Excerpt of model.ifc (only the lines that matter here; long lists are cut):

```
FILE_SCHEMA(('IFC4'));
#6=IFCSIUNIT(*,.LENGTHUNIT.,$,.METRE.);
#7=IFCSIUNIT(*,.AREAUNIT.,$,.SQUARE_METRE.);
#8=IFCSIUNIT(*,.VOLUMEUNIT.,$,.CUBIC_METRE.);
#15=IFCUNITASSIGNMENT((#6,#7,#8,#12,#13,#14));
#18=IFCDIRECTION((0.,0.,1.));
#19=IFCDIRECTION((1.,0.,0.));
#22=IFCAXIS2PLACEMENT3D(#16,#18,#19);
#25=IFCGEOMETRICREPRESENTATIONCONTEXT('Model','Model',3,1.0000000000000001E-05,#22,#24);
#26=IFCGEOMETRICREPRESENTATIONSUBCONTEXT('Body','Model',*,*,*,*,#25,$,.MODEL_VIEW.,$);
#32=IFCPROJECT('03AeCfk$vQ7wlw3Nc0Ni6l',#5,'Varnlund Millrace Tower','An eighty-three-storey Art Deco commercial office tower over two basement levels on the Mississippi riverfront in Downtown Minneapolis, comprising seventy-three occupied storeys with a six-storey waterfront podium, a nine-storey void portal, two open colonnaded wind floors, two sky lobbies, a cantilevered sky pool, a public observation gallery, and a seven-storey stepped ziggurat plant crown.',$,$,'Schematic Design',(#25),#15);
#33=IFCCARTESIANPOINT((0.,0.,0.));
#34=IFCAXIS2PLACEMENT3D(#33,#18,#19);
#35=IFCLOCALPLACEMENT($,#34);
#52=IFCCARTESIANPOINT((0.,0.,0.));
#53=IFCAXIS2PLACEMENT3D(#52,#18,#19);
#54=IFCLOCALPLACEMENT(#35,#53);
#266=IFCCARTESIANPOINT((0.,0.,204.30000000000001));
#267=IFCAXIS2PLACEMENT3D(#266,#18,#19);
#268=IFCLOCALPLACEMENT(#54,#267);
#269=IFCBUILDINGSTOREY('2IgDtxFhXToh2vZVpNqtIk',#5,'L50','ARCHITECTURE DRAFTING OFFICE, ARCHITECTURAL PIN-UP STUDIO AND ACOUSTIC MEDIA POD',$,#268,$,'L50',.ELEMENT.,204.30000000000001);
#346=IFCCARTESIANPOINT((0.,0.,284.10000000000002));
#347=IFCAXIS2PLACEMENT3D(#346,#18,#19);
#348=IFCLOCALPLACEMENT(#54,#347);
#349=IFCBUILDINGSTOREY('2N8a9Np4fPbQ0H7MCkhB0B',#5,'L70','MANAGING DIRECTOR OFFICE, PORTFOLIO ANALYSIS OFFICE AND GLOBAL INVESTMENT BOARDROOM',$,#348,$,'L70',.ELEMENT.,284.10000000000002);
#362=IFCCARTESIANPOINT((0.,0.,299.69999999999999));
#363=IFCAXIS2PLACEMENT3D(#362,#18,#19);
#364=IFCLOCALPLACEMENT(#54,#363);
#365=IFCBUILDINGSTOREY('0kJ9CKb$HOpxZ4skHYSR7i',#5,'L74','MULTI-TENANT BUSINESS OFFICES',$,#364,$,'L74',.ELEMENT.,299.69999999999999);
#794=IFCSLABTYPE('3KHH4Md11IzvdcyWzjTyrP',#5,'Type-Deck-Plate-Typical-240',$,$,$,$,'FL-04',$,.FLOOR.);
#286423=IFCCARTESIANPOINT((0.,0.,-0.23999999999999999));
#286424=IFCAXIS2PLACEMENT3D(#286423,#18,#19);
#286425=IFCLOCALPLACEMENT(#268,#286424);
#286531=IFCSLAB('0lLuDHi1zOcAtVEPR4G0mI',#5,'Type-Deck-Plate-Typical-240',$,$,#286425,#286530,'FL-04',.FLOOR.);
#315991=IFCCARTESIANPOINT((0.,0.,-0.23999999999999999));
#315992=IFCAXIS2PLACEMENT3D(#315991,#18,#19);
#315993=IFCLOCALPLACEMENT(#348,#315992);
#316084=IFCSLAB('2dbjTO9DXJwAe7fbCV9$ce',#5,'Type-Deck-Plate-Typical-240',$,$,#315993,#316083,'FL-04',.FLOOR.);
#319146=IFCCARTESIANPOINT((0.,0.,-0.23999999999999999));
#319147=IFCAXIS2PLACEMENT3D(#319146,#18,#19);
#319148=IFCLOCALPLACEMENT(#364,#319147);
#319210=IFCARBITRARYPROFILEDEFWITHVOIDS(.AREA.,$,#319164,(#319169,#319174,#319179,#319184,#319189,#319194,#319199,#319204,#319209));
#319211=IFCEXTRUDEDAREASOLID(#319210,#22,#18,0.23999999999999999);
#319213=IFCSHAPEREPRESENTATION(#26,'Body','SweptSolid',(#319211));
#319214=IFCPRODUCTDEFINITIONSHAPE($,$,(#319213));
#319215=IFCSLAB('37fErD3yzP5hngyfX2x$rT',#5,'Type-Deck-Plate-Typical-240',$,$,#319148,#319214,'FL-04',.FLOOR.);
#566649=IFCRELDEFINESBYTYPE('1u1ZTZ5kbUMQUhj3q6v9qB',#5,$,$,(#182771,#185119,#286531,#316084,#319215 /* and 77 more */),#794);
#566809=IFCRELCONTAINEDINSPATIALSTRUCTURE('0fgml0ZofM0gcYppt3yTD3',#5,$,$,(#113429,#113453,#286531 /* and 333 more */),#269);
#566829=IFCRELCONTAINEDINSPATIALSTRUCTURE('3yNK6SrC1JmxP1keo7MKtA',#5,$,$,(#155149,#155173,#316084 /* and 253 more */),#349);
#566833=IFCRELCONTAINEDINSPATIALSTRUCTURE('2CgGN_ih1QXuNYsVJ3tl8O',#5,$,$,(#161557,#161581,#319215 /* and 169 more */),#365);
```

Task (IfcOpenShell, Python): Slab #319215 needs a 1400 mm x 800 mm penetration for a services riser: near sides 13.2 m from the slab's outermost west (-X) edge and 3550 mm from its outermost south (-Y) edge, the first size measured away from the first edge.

```python
import numpy as np
import ifcopenshell
import ifcopenshell.api.feature
import ifcopenshell.api.geometry
import ifcopenshell.api.root
import ifcopenshell.geom
import ifcopenshell.util.placement
import ifcopenshell.util.representation
import ifcopenshell.util.shape
import ifcopenshell.util.unit

model = ifcopenshell.open("model.ifc")
unit_scale = ifcopenshell.util.unit.calculate_unit_scale(model)
settings = ifcopenshell.geom.settings()


def volume(element):
    """Net volume in cubic metres, openings subtracted."""
    shape = ifcopenshell.geom.create_shape(settings, element)
    return ifcopenshell.util.shape.get_volume(shape.geometry)


slab = model.by_guid("37fErD3yzP5hngyfX2x$rT")
before = volume(slab)

# Extent in the slab's own axes, in metres. The edges named are its -X and -Y sides.
slab_shape = ifcopenshell.geom.create_shape(settings, slab)
vertices = ifcopenshell.util.shape.get_vertices(slab_shape.geometry)
x_min, y_min, bottom = vertices.min(axis=0)
top = vertices[:, 2].max()

opening = ifcopenshell.api.root.create_entity(model, ifc_class="IfcOpeningElement", name="Services riser opening", predefined_type="OPENING")
context = ifcopenshell.util.representation.get_context(model, "Model", "Body", "MODEL_VIEW")
width, depth = 1.4, 0.8
outline = [(0.0, 0.0), (width, 0.0), (width, depth), (0.0, depth), (0.0, 0.0)]
# Overshoot both faces by 50 mm so the cut is clean.
shape = ifcopenshell.api.geometry.add_slab_representation(
    model, context=context, depth=top - bottom + 0.1, polyline=outline
)
ifcopenshell.api.geometry.assign_representation(model, product=opening, representation=shape)

matrix = ifcopenshell.util.placement.get_local_placement(slab.ObjectPlacement)
matrix[:, 3] = matrix @ np.append(np.array([x_min + 13.2, y_min + 3.55, bottom - 0.05]) / unit_scale, 1.0)
ifcopenshell.api.geometry.edit_object_placement(model, product=opening, matrix=matrix, is_si=False)
ifcopenshell.api.feature.add_feature(model, feature=opening, element=slab)

after = volume(slab)

print(f"slab volume {before:.3f} -> {after:.3f} m3")

model.write("model_edited.ifc")
```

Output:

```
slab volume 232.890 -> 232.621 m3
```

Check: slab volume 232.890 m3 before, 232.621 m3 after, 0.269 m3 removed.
